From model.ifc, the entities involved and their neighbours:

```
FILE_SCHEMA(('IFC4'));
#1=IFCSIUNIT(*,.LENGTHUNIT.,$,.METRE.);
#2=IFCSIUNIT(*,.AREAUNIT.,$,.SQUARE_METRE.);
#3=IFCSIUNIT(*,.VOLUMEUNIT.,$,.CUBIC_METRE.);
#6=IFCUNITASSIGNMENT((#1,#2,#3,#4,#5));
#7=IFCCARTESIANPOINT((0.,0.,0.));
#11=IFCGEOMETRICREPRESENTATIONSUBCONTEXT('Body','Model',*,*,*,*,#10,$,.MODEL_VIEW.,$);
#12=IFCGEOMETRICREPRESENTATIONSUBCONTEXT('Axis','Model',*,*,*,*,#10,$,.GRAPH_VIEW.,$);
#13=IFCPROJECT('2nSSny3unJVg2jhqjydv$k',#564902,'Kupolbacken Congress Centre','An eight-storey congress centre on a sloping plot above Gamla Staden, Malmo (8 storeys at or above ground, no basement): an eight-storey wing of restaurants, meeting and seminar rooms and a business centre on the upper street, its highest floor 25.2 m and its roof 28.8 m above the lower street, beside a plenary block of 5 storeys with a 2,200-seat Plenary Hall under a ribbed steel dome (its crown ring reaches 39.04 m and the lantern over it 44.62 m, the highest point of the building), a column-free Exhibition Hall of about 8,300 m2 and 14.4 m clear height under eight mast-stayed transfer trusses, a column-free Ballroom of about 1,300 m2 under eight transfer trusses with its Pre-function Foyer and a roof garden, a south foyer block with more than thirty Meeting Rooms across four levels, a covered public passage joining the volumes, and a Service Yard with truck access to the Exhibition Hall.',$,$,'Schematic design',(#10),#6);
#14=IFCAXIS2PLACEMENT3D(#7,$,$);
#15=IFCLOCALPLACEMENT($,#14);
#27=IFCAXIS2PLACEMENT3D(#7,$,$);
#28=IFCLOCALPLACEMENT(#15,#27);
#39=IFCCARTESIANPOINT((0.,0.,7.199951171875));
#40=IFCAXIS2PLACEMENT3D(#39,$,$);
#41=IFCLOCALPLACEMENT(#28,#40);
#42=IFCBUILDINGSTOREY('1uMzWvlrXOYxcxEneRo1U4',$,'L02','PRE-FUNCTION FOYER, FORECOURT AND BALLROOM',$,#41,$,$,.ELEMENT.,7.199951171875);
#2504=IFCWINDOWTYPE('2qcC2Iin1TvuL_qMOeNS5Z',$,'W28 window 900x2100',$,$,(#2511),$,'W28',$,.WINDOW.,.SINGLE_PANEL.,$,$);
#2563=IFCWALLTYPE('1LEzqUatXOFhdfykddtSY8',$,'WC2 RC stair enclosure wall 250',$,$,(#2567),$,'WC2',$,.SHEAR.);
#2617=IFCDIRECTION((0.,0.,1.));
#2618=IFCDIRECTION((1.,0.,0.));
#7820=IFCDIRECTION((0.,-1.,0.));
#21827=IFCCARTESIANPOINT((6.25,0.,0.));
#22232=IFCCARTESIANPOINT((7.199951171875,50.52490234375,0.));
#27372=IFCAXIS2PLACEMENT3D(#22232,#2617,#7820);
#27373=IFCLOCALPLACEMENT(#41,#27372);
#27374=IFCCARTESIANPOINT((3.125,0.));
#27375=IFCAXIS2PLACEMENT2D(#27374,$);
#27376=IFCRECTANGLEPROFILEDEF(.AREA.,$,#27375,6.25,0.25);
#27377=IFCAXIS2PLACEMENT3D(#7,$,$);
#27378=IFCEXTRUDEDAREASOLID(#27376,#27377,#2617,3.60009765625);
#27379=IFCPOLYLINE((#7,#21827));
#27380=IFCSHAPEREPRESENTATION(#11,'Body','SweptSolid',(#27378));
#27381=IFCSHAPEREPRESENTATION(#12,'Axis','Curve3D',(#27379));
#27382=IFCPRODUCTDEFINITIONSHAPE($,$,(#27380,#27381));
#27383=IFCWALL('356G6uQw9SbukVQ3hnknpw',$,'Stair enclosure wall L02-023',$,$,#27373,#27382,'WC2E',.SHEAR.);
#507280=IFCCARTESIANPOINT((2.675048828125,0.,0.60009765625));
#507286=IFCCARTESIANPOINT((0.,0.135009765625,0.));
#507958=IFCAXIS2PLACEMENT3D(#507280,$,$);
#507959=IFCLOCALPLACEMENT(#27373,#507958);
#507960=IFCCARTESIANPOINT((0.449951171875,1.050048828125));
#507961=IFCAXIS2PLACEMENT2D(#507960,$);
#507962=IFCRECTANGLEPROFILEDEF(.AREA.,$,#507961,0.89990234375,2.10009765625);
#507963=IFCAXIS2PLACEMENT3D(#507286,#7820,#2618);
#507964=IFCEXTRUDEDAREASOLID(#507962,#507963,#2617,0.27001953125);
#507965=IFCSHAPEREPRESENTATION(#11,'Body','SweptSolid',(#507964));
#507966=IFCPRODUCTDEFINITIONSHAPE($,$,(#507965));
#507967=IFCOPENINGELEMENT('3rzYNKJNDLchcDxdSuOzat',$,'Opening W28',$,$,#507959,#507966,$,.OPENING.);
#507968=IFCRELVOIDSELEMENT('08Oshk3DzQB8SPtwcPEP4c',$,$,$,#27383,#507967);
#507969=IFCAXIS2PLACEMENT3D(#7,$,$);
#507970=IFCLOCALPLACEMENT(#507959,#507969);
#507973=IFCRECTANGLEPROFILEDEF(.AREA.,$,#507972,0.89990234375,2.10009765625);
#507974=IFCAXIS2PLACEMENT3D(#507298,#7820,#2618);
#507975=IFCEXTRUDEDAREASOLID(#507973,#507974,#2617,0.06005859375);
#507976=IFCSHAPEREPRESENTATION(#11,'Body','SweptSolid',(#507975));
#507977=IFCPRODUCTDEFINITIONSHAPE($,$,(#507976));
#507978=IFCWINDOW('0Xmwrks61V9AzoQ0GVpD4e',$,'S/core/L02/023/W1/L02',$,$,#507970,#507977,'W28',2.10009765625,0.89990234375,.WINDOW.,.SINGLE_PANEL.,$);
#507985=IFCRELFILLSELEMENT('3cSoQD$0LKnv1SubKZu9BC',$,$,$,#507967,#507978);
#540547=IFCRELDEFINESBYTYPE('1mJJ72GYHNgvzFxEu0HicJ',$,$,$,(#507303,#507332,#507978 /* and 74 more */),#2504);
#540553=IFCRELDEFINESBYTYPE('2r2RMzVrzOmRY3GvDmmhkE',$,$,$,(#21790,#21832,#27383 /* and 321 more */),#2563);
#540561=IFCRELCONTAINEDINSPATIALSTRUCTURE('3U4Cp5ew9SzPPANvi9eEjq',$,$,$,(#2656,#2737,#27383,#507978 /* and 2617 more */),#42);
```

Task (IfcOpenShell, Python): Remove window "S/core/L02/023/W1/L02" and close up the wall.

```python
import ifcopenshell
import ifcopenshell.api.feature
import ifcopenshell.api.root
import ifcopenshell.geom
import ifcopenshell.util.shape

model = ifcopenshell.open("model.ifc")
settings = ifcopenshell.geom.settings()


def volume(element):
    """Net volume in cubic metres, openings subtracted."""
    shape = ifcopenshell.geom.create_shape(settings, element)
    return ifcopenshell.util.shape.get_volume(shape.geometry)


window = model.by_id(507978)
opening = window.FillsVoids[0].RelatingOpeningElement
wall = opening.VoidsElements[0].RelatingBuildingElement
before = volume(wall)

ifcopenshell.api.root.remove_product(model, product=window)
ifcopenshell.api.feature.remove_feature(model, feature=opening)

after = volume(wall)

print(f"wall volume {before:.3f} -> {after:.3f} m3")

model.write("model_rev.ifc")
```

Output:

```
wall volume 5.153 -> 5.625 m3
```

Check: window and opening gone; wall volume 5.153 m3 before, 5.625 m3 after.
